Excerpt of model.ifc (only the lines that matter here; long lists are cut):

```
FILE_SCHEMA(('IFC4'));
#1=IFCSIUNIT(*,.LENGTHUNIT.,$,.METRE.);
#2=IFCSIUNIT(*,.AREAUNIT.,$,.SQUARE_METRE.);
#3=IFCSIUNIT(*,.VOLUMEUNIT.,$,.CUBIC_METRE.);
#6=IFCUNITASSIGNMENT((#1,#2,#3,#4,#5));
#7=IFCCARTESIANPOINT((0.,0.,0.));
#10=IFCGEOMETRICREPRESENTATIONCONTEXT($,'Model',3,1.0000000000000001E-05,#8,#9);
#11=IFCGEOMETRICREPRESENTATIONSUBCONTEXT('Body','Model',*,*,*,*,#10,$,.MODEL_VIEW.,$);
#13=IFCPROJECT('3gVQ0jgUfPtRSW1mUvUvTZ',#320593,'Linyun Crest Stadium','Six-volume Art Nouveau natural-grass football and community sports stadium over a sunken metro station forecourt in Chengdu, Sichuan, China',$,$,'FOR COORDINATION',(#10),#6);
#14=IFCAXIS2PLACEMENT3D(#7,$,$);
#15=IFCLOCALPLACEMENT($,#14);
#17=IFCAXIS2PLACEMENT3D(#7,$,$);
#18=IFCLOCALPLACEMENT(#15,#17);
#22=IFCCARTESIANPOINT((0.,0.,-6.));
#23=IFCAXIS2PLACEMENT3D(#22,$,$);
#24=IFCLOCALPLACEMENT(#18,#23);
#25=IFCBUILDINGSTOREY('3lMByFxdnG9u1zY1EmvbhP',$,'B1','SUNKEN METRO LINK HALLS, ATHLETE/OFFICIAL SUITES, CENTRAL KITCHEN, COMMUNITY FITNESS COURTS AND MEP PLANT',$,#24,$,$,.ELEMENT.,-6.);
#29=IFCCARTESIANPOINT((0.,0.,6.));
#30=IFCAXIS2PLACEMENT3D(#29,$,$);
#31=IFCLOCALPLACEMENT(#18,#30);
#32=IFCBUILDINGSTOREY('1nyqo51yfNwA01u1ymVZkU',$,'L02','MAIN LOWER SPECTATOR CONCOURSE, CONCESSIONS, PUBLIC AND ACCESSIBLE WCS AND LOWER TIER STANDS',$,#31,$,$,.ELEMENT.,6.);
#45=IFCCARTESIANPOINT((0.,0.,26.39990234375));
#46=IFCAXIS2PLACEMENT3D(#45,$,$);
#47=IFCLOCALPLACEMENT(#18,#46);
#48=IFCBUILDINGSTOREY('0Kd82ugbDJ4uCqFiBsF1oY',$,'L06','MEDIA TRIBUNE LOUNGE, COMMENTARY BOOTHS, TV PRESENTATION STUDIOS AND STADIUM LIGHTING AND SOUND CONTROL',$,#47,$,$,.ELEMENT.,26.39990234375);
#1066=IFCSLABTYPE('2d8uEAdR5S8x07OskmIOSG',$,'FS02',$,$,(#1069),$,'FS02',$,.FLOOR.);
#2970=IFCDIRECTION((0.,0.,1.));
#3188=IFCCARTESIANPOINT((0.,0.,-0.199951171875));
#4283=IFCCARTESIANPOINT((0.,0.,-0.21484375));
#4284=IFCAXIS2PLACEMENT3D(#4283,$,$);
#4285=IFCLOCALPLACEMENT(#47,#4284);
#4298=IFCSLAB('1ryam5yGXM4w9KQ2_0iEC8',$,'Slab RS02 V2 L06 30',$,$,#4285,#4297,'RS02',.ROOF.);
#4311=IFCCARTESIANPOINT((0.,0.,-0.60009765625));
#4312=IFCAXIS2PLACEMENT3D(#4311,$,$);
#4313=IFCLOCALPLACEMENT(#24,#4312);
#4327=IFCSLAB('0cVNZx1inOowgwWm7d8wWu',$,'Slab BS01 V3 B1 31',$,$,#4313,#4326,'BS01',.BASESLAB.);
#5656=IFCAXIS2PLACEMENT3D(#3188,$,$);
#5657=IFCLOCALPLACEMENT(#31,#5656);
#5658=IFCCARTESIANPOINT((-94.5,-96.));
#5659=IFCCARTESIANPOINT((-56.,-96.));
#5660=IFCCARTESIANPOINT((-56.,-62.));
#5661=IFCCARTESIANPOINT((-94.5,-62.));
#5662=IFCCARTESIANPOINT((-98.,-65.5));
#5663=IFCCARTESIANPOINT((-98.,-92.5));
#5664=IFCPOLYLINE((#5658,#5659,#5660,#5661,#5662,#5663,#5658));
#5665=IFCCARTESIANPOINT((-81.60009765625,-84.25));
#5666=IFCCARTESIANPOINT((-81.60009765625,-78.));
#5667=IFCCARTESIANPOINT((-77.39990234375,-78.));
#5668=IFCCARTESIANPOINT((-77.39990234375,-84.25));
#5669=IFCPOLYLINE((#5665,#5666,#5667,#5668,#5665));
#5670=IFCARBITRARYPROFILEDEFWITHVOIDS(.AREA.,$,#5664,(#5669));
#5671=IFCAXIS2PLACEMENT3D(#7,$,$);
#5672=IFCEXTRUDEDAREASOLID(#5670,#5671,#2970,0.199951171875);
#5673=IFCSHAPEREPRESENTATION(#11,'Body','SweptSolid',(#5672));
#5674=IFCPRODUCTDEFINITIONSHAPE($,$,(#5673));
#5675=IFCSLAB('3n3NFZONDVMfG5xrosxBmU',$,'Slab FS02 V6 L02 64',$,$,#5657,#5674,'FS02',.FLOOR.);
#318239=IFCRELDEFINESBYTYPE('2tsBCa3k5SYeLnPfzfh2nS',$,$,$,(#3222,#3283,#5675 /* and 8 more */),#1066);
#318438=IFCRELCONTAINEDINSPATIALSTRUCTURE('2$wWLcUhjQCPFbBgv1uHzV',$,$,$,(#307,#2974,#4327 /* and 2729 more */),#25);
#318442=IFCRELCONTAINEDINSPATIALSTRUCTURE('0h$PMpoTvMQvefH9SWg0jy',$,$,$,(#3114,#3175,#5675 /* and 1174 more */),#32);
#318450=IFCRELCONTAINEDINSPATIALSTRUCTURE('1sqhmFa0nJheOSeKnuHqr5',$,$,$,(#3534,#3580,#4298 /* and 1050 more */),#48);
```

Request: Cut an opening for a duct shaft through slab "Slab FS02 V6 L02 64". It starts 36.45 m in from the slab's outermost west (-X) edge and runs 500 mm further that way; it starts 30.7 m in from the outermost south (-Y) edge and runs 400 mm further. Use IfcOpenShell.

```python
import numpy as np
import ifcopenshell
import ifcopenshell.api.feature
import ifcopenshell.api.geometry
import ifcopenshell.api.root
import ifcopenshell.geom
import ifcopenshell.util.placement
import ifcopenshell.util.representation
import ifcopenshell.util.shape
import ifcopenshell.util.unit

model = ifcopenshell.open("model.ifc")
unit_scale = ifcopenshell.util.unit.calculate_unit_scale(model)
settings = ifcopenshell.geom.settings()


def volume(element):
    """Net volume in cubic metres, openings subtracted."""
    shape = ifcopenshell.geom.create_shape(settings, element)
    return ifcopenshell.util.shape.get_volume(shape.geometry)


slab = model.by_id(5675)
before = volume(slab)

# Extent in the slab's own axes, in metres. The edges named are its -X and -Y sides.
slab_shape = ifcopenshell.geom.create_shape(settings, slab)
vertices = ifcopenshell.util.shape.get_vertices(slab_shape.geometry)
x_min, y_min, bottom = vertices.min(axis=0)
top = vertices[:, 2].max()

opening = ifcopenshell.api.root.create_entity(model, ifc_class="IfcOpeningElement", name="Duct shaft opening", predefined_type="OPENING")
context = ifcopenshell.util.representation.get_context(model, "Model", "Body", "MODEL_VIEW")
width, depth = 0.5, 0.4
outline = [(0.0, 0.0), (width, 0.0), (width, depth), (0.0, depth), (0.0, 0.0)]
# Overshoot both faces by 50 mm so the cut is clean.
shape = ifcopenshell.api.geometry.add_slab_representation(
    model, context=context, depth=top - bottom + 0.1, polyline=outline
)
ifcopenshell.api.geometry.assign_representation(model, product=opening, representation=shape)

matrix = ifcopenshell.util.placement.get_local_placement(slab.ObjectPlacement)
matrix[:, 3] = matrix @ np.append(np.array([x_min + 36.45, y_min + 30.7, bottom - 0.05]) / unit_scale, 1.0)
ifcopenshell.api.geometry.edit_object_placement(model, product=opening, matrix=matrix, is_si=False)
ifcopenshell.api.feature.add_feature(model, feature=opening, element=slab)

after = volume(slab)

print(f"slab volume {before:.3f} -> {after:.3f} m3")

model.write("model_v2.ifc")
```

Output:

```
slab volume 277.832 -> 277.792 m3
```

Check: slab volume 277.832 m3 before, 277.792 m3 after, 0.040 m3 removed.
